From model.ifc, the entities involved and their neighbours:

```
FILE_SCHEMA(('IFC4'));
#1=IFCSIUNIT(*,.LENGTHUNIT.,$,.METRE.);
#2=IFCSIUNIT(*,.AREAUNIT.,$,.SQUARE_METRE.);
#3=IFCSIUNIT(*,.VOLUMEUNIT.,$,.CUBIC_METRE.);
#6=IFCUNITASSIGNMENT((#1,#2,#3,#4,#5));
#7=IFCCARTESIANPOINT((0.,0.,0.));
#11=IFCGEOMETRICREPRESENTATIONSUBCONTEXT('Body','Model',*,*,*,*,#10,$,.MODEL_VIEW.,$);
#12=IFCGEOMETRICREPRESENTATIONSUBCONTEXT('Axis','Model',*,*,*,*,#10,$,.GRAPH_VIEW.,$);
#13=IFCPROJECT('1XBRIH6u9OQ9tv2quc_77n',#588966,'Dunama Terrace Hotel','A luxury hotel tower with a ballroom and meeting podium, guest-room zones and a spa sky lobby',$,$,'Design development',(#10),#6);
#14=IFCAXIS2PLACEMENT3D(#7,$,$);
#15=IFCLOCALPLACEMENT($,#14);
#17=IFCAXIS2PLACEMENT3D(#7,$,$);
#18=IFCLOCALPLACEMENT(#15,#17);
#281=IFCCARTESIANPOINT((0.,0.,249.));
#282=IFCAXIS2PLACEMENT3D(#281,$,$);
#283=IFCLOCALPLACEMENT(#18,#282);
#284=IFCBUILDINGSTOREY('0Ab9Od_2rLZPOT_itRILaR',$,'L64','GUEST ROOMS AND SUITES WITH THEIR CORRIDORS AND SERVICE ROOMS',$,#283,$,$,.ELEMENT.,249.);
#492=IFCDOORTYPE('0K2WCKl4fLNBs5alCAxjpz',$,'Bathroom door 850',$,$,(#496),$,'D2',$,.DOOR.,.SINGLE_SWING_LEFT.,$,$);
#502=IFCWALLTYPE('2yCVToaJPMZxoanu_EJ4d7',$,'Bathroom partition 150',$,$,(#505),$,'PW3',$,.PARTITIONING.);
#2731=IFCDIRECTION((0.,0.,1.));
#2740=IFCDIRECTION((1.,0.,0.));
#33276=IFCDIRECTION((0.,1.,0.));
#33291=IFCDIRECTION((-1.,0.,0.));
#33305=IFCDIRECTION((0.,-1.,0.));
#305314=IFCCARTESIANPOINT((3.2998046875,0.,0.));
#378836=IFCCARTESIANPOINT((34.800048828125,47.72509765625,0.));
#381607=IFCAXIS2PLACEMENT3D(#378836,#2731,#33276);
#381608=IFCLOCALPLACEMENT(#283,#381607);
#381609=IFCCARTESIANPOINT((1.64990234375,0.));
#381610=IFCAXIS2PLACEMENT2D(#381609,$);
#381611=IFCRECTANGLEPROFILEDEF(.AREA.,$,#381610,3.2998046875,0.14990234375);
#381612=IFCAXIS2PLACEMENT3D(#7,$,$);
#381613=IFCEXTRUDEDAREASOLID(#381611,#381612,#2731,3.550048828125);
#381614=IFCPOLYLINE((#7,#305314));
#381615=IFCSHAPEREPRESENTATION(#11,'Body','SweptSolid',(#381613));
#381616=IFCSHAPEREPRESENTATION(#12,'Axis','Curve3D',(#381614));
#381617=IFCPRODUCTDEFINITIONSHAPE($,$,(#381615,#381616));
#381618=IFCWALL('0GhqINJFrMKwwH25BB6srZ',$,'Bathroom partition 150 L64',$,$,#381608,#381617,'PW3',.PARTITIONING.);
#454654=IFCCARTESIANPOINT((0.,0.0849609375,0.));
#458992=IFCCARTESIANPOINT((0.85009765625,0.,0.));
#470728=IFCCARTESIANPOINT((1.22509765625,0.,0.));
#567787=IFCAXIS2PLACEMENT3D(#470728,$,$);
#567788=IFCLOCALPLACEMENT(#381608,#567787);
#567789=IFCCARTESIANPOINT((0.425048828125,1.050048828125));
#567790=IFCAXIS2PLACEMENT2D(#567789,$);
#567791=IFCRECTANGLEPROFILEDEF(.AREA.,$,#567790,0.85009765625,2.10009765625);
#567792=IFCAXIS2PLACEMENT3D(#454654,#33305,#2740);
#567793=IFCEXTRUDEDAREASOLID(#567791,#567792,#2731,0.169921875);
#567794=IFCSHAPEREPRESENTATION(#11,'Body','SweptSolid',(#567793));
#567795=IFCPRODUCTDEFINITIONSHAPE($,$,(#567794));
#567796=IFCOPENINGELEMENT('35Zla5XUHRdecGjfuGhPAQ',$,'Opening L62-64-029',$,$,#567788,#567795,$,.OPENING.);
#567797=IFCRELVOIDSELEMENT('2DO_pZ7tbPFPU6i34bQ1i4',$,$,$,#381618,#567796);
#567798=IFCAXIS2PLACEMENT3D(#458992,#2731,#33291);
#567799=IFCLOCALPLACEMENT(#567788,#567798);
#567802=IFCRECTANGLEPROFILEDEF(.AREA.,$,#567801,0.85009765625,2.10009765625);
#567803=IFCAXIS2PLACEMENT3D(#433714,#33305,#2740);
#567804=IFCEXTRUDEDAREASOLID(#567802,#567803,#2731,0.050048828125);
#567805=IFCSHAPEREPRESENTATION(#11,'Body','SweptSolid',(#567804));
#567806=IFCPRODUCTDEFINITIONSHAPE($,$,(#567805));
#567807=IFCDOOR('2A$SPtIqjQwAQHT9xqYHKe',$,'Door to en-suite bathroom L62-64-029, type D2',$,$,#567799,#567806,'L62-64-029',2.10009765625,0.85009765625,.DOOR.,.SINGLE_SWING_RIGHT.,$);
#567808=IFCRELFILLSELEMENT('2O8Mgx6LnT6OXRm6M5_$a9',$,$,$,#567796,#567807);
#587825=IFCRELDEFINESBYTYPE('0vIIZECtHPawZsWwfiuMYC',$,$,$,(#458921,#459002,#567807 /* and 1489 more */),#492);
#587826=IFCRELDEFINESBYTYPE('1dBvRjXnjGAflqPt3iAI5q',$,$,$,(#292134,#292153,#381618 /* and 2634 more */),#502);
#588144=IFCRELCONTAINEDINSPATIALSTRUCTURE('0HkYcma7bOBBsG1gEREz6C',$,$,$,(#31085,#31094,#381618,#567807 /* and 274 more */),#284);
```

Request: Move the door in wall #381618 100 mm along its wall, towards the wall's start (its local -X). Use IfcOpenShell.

```python
import ifcopenshell
import ifcopenshell.api.geometry
import ifcopenshell.util.placement
import ifcopenshell.util.unit

model = ifcopenshell.open("model.ifc")
unit_scale = ifcopenshell.util.unit.calculate_unit_scale(model)

door = model.by_id(567807)
opening = door.FillsVoids[0].RelatingOpeningElement
wall = opening.VoidsElements[0].RelatingBuildingElement

wall_matrix = ifcopenshell.util.placement.get_local_placement(wall.ObjectPlacement)
shift = wall_matrix[:3, 0] * -0.1 / unit_scale
before = ifcopenshell.util.placement.get_local_placement(door.ObjectPlacement)[:3, 3].copy()

# The door is placed relative to its opening, so it follows when the opening moves.
matrix = ifcopenshell.util.placement.get_local_placement(opening.ObjectPlacement)
matrix[:3, 3] += shift
ifcopenshell.api.geometry.edit_object_placement(
    model, product=opening, matrix=matrix, is_si=False, should_transform_children=True
)

after = ifcopenshell.util.placement.get_local_placement(door.ObjectPlacement)[:3, 3]
print("door moved by", (after - before).round(3) + 0.0)

model.write("model_rev.ifc")
```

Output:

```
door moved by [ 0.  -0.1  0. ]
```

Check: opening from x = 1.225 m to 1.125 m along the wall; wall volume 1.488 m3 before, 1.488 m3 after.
